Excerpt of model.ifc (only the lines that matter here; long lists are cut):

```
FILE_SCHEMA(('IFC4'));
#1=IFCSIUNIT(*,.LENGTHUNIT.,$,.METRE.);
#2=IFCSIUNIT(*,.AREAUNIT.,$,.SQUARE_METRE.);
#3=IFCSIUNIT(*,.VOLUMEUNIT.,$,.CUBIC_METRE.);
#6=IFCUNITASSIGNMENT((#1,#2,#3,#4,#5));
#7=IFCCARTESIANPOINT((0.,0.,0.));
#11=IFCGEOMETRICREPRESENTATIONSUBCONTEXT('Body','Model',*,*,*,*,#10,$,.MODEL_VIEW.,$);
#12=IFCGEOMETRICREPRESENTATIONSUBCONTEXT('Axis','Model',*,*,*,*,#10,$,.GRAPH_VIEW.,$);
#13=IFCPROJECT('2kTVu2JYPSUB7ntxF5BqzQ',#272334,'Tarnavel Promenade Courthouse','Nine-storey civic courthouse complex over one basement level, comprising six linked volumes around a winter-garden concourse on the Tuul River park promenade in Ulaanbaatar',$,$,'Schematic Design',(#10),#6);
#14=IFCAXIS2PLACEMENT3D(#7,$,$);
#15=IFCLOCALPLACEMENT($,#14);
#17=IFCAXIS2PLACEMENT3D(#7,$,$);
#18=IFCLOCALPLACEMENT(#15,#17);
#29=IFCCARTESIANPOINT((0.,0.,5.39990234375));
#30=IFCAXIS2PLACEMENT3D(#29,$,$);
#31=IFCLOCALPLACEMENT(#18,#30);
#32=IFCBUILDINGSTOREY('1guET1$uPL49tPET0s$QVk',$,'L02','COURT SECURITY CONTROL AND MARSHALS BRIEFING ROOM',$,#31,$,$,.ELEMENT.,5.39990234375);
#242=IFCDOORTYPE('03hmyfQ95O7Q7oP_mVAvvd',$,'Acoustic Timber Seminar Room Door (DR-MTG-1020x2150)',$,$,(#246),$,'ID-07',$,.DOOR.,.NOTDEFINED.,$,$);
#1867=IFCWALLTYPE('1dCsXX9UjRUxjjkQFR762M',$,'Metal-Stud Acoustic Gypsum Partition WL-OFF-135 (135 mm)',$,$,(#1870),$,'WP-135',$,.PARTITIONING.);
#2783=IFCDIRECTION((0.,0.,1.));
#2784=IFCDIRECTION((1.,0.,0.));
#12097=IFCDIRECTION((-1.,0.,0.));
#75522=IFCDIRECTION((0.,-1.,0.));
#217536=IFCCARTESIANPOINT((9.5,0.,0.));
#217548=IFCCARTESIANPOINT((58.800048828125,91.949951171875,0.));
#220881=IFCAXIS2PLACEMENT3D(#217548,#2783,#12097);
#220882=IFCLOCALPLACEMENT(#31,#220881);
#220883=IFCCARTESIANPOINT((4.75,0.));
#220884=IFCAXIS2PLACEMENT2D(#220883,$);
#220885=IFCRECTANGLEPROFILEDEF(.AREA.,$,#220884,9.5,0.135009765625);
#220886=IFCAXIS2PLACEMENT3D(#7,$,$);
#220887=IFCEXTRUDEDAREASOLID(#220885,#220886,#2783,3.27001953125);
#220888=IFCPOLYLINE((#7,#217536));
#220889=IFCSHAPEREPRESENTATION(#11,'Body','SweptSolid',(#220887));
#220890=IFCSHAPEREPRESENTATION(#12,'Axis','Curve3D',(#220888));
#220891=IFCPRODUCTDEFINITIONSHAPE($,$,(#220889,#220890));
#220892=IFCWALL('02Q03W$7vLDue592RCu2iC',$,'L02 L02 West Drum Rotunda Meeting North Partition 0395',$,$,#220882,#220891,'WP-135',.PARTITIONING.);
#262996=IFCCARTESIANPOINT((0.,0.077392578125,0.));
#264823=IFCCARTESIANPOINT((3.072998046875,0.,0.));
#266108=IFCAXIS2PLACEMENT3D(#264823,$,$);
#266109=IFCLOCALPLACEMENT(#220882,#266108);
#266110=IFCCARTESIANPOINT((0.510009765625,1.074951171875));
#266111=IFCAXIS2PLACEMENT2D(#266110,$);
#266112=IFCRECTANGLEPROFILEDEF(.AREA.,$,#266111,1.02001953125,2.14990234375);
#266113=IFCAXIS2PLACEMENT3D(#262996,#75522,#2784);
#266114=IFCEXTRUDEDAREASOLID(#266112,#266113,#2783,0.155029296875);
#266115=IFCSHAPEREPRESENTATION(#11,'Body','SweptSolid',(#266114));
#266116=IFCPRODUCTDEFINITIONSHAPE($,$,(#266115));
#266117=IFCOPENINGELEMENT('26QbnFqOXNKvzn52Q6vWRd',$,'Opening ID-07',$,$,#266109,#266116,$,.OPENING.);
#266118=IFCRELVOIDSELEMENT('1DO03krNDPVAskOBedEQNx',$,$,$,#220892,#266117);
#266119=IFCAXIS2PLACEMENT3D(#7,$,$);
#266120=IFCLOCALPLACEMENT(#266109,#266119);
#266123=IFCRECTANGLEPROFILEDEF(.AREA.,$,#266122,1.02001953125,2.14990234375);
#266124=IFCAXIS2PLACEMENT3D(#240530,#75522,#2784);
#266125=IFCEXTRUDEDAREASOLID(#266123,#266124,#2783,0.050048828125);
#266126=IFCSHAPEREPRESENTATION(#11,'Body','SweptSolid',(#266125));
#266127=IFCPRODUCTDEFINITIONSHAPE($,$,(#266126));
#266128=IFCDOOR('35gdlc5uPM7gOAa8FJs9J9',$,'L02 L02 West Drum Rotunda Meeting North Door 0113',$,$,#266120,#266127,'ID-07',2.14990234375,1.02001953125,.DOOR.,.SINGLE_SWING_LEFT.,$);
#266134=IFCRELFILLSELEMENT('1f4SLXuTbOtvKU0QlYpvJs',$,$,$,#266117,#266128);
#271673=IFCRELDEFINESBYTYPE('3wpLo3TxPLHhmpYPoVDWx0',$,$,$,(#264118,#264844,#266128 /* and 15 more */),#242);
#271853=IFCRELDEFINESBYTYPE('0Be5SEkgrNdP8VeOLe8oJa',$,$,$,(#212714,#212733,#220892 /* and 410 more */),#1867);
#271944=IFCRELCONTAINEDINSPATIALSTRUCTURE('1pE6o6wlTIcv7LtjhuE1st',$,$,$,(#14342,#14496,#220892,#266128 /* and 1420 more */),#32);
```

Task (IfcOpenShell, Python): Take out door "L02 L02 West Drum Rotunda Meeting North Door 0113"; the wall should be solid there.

```python
import ifcopenshell
import ifcopenshell.api.feature
import ifcopenshell.api.root
import ifcopenshell.geom
import ifcopenshell.util.shape

model = ifcopenshell.open("model.ifc")
settings = ifcopenshell.geom.settings()


def volume(element):
    """Net volume in cubic metres, openings subtracted."""
    shape = ifcopenshell.geom.create_shape(settings, element)
    return ifcopenshell.util.shape.get_volume(shape.geometry)


door = model.by_id(266128)
opening = door.FillsVoids[0].RelatingOpeningElement
wall = opening.VoidsElements[0].RelatingBuildingElement
before = volume(wall)

ifcopenshell.api.root.remove_product(model, product=door)
ifcopenshell.api.feature.remove_feature(model, feature=opening)

after = volume(wall)

print(f"wall volume {before:.3f} -> {after:.3f} m3")

model.write("model_rev.ifc")
```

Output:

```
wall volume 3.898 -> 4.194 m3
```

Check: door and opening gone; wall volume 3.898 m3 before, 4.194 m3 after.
